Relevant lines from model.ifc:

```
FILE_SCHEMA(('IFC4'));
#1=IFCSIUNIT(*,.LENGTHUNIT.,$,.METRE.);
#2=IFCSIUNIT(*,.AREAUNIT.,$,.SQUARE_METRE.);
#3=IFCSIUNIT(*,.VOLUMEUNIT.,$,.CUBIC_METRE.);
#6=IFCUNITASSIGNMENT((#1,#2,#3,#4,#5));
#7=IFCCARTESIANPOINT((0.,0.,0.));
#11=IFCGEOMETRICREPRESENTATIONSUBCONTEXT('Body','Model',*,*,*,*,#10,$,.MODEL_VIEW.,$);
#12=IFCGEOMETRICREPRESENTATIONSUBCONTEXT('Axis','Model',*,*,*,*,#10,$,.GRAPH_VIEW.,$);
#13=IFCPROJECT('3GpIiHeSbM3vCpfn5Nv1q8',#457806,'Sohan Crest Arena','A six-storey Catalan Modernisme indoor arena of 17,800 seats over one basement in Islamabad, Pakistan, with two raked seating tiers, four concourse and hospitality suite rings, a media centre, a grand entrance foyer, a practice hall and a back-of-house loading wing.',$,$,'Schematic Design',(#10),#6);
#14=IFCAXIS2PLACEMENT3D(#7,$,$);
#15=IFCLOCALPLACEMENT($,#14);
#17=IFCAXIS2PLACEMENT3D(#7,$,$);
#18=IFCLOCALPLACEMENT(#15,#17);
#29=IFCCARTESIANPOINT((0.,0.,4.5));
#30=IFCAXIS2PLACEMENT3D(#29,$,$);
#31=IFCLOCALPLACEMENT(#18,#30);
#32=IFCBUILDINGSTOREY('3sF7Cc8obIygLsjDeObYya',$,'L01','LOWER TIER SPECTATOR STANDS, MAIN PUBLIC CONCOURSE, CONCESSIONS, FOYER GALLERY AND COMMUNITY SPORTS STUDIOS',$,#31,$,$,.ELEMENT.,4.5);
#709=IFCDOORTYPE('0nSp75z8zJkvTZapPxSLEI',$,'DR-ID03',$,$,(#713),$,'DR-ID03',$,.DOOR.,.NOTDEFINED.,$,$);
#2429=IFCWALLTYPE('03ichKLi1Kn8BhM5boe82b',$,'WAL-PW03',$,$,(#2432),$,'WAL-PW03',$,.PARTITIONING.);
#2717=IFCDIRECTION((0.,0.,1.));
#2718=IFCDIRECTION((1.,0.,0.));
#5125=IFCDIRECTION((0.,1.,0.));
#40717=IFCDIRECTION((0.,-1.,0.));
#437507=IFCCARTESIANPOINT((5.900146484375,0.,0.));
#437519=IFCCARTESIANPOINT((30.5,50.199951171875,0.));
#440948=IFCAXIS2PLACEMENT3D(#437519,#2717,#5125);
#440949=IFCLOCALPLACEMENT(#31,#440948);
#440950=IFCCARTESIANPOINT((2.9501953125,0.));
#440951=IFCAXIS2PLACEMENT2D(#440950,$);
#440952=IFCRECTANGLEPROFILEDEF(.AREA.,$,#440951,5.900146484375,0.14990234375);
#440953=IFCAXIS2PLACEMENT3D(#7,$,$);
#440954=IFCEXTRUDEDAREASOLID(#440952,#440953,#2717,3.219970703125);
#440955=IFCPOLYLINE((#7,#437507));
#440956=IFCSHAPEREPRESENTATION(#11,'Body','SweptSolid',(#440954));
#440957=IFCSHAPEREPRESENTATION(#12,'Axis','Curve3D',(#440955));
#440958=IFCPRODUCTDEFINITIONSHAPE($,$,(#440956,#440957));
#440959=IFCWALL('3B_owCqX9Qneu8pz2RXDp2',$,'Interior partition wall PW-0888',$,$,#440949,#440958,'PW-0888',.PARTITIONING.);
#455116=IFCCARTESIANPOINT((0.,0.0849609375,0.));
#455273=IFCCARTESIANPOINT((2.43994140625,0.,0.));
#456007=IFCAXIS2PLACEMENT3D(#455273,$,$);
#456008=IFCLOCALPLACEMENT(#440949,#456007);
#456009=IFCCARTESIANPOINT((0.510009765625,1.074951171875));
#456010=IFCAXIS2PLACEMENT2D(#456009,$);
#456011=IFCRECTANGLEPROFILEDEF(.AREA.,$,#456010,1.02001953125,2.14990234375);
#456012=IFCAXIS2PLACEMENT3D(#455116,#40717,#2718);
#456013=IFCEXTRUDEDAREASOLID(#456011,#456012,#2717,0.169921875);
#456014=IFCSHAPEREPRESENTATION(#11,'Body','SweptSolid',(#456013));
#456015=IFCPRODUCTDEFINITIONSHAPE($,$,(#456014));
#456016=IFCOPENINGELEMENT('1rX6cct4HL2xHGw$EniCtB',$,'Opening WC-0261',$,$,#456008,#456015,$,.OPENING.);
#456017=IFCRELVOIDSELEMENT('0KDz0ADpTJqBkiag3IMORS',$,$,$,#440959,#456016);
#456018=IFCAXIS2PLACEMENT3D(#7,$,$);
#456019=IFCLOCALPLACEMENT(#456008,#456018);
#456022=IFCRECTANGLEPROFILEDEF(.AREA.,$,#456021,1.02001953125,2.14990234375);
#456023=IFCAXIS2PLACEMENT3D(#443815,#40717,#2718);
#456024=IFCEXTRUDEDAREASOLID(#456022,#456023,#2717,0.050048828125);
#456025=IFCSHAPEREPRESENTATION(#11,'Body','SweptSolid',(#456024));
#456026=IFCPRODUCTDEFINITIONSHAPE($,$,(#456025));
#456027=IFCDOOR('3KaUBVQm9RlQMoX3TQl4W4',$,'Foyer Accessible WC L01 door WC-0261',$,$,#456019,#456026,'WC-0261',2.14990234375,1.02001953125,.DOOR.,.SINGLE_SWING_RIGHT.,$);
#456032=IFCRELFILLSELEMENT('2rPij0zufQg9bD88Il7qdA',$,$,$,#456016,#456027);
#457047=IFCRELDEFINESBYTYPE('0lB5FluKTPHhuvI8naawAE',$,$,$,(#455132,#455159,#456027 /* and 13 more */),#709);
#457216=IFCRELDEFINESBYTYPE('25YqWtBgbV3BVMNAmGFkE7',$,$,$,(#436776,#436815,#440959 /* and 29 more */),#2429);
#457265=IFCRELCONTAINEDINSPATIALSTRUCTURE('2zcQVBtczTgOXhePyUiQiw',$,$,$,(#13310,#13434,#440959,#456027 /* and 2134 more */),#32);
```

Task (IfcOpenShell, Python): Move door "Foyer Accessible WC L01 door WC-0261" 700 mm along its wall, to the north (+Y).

```python
import ifcopenshell
import ifcopenshell.api.geometry
import ifcopenshell.util.placement
import ifcopenshell.util.unit

model = ifcopenshell.open("model.ifc")
unit_scale = ifcopenshell.util.unit.calculate_unit_scale(model)

door = model.by_guid("3KaUBVQm9RlQMoX3TQl4W4")
opening = door.FillsVoids[0].RelatingOpeningElement
wall = opening.VoidsElements[0].RelatingBuildingElement

wall_matrix = ifcopenshell.util.placement.get_local_placement(wall.ObjectPlacement)
shift = wall_matrix[:3, 0] * 0.7 / unit_scale
before = ifcopenshell.util.placement.get_local_placement(door.ObjectPlacement)[:3, 3].copy()

# The door is placed relative to its opening, so it follows when the opening moves.
matrix = ifcopenshell.util.placement.get_local_placement(opening.ObjectPlacement)
matrix[:3, 3] += shift
ifcopenshell.api.geometry.edit_object_placement(
    model, product=opening, matrix=matrix, is_si=False, should_transform_children=True
)

after = ifcopenshell.util.placement.get_local_placement(door.ObjectPlacement)[:3, 3]
print("door moved by", (after - before).round(3) + 0.0)

model.write("model_v2.ifc")
```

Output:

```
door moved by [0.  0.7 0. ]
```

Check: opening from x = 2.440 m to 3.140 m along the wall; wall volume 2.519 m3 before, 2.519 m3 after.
